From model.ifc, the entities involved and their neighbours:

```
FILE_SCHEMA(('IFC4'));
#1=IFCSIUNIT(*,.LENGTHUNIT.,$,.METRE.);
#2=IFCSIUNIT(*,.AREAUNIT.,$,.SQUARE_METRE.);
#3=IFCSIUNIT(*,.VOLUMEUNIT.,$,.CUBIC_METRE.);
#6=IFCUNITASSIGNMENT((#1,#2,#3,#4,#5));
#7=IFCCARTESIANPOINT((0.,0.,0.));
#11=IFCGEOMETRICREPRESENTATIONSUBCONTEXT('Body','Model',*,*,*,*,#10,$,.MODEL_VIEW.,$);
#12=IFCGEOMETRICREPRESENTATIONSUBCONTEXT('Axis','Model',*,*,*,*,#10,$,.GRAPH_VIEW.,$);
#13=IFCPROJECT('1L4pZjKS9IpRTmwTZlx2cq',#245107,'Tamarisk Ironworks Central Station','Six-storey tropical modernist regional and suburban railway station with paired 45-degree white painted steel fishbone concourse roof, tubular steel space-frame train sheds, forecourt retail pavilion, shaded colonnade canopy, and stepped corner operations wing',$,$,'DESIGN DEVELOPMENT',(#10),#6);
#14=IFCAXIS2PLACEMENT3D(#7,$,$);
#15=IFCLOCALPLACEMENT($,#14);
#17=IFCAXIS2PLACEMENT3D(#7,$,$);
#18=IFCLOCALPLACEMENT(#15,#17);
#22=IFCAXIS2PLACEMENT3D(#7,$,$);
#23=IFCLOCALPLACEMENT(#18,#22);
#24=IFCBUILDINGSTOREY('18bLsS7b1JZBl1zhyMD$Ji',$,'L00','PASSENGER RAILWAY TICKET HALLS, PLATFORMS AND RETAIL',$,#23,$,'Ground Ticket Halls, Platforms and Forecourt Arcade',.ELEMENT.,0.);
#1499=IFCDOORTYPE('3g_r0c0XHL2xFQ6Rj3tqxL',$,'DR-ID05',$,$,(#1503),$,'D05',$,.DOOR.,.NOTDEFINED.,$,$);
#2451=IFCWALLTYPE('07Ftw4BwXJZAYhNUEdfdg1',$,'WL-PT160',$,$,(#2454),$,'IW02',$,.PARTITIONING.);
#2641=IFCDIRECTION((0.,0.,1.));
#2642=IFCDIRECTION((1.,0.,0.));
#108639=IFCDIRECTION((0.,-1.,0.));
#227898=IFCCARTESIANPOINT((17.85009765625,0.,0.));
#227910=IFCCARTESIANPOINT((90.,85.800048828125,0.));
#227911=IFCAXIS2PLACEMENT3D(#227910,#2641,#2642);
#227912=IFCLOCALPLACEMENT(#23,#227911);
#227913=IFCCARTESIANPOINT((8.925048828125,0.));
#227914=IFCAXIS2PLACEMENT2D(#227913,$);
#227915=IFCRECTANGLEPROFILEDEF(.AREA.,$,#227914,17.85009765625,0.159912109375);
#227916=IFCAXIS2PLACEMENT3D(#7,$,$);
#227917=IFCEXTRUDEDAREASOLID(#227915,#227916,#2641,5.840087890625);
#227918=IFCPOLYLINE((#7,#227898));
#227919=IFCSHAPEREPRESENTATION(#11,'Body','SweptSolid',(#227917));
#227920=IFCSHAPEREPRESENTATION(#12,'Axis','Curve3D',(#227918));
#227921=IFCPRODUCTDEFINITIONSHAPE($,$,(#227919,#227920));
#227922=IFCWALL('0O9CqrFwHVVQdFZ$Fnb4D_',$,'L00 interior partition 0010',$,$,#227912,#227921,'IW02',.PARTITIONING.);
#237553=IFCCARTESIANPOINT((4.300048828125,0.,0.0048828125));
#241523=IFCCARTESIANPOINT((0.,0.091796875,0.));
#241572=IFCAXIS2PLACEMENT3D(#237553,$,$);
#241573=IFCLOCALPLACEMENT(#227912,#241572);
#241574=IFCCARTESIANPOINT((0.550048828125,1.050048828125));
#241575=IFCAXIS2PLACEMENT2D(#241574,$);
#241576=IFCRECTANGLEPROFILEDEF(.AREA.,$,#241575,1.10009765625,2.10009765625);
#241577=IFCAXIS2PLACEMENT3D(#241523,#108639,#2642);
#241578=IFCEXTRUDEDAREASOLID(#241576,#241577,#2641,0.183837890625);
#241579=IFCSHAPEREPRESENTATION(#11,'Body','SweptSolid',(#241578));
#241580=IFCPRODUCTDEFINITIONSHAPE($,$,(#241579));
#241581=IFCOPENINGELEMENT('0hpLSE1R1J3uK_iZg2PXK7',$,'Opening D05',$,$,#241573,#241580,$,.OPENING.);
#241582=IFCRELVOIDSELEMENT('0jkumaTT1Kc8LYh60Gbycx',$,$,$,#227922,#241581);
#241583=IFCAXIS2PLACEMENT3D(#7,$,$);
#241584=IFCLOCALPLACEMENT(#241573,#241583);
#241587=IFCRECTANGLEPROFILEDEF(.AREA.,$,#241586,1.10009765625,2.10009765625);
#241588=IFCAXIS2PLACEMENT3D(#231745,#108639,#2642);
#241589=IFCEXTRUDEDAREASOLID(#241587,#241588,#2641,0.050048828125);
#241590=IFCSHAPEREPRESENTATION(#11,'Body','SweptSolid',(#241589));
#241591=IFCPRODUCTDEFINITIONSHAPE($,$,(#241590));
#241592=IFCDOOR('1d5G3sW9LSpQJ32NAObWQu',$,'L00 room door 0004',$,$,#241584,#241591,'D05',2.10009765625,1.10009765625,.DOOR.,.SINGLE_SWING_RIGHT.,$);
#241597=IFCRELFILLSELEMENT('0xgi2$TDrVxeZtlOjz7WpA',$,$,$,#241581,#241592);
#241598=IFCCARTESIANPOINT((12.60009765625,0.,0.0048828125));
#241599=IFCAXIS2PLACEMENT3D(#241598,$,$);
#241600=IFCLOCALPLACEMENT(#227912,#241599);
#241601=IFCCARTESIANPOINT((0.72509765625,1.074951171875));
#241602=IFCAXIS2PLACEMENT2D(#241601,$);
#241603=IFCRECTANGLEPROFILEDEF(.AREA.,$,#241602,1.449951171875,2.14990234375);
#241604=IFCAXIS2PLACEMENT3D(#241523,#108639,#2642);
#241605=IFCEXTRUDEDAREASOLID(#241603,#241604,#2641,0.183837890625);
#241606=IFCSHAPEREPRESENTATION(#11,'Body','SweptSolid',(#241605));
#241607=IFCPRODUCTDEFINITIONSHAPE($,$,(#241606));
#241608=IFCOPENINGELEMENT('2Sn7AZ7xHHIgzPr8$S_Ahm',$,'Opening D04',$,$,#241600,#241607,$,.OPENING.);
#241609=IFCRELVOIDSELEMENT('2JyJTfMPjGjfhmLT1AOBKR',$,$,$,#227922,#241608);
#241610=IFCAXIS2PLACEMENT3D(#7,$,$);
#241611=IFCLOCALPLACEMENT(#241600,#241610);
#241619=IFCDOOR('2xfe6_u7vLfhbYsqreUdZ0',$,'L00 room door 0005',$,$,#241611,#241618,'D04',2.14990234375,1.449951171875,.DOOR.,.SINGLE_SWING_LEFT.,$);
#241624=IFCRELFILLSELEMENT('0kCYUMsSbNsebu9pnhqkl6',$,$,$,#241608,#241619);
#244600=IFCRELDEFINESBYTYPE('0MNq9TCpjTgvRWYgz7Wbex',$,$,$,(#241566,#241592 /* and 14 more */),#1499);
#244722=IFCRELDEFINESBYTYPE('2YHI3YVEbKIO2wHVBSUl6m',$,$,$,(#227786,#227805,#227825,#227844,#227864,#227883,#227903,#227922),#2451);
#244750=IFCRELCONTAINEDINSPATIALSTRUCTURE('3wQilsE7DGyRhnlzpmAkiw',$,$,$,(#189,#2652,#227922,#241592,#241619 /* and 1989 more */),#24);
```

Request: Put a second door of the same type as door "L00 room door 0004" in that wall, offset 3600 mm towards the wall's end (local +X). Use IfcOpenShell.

```python
import ifcopenshell
import ifcopenshell.api.feature
import ifcopenshell.api.geometry
import ifcopenshell.api.root
import ifcopenshell.geom
import ifcopenshell.util.element
import ifcopenshell.util.placement
import ifcopenshell.util.shape

model = ifcopenshell.open("model.ifc")
settings = ifcopenshell.geom.settings()


def volume(element):
    """Net volume in cubic metres, openings subtracted."""
    shape = ifcopenshell.geom.create_shape(settings, element)
    return ifcopenshell.util.shape.get_volume(shape.geometry)


door = model.by_guid("1d5G3sW9LSpQJ32NAObWQu")
opening = door.FillsVoids[0].RelatingOpeningElement
wall = opening.VoidsElements[0].RelatingBuildingElement
before = volume(wall)
shift = ifcopenshell.util.placement.get_local_placement(wall.ObjectPlacement)[:3, 0] * 3.6

# copy_class copies the void relationship, type, container and properties, but no geometry.
new_opening = ifcopenshell.api.root.copy_class(model, product=opening)
new_opening.Representation = ifcopenshell.util.element.copy_deep(
    model, opening.Representation, exclude=["IfcGeometricRepresentationContext", "IfcRepresentationMap"]
)
new_door = ifcopenshell.api.root.copy_class(model, product=door)
new_door.Representation = ifcopenshell.util.element.copy_deep(
    model, door.Representation, exclude=["IfcGeometricRepresentationContext", "IfcRepresentationMap"]
)
new_door.Tag = None
ifcopenshell.api.feature.add_filling(model, opening=new_opening, element=new_door)

for old, new in ((opening, new_opening), (door, new_door)):
    matrix = ifcopenshell.util.placement.get_local_placement(old.ObjectPlacement)
    matrix[:3, 3] += shift
    ifcopenshell.api.geometry.edit_object_placement(model, product=new, matrix=matrix, is_si=False)

after = volume(wall)

print(f"wall volume {before:.3f} -> {after:.3f} m3")

model.write("model-out.ifc")
```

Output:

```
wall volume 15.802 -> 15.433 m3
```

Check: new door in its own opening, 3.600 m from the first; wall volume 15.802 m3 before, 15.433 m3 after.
